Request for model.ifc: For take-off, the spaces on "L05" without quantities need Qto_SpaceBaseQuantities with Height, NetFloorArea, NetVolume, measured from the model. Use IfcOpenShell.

First a look at what the model holds.

```python
import ifcopenshell
import ifcopenshell.util.element
import ifcopenshell.util.unit

model = ifcopenshell.open("model.ifc")
print(model.schema)
for unit_type in ("LENGTHUNIT", "AREAUNIT", "VOLUMEUNIT"):
    print(unit_type, ifcopenshell.util.unit.calculate_unit_scale(model, unit_type))
storey = next(s for s in model.by_type("IfcBuildingStorey") if s.Name == "L05")
spaces = [e for e in ifcopenshell.util.element.get_decomposition(storey) if e.is_a("IfcSpace")]
for e in sorted(spaces, key=lambda e: e.id()):
    print(e.id(), e.is_a(), e.Name, list(ifcopenshell.util.element.get_psets(e, qtos_only=True)), sep=" | ")
```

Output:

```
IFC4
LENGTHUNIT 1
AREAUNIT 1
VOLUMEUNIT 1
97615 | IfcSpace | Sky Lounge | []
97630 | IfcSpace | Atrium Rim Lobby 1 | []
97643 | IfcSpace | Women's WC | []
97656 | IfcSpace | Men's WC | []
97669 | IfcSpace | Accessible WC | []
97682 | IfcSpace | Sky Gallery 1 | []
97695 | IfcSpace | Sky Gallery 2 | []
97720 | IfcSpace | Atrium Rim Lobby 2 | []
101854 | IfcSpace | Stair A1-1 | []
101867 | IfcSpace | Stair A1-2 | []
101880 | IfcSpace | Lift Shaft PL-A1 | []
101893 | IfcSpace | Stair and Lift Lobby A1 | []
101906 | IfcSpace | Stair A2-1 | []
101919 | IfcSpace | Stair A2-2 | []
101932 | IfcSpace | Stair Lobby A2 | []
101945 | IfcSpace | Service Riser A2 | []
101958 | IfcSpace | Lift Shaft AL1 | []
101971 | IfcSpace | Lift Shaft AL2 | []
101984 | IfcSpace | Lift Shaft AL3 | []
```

```python
import ifcopenshell
import ifcopenshell.api.pset
import ifcopenshell.geom
import ifcopenshell.util.element
import ifcopenshell.util.shape
import ifcopenshell.util.unit

model = ifcopenshell.open("model.ifc")
unit_scale = ifcopenshell.util.unit.calculate_unit_scale(model)
area_scale = ifcopenshell.util.unit.calculate_unit_scale(model, "AREAUNIT")
volume_scale = ifcopenshell.util.unit.calculate_unit_scale(model, "VOLUMEUNIT")
settings = ifcopenshell.geom.settings()

storey = next(s for s in model.by_type("IfcBuildingStorey") if s.Name == "L05")
spaces = [e for e in ifcopenshell.util.element.get_decomposition(storey) if e.is_a("IfcSpace")]

for e in sorted(spaces, key=lambda e: e.id()):
    if ifcopenshell.util.element.get_psets(e, qtos_only=True, should_inherit=False):
        continue
    # Geometry comes back in metres, in the element's own axes.
    shape = ifcopenshell.geom.create_shape(settings, e)
    values = {
        "Height": ifcopenshell.util.shape.get_z(shape.geometry) / unit_scale,
        "NetFloorArea": ifcopenshell.util.shape.get_footprint_area(shape.geometry) / area_scale,
        "NetVolume": ifcopenshell.util.shape.get_volume(shape.geometry) / volume_scale,
    }
    qto = ifcopenshell.api.pset.add_qto(model, product=e, name="Qto_SpaceBaseQuantities")
    ifcopenshell.api.pset.edit_qto(model, qto=qto, properties=values)
    print(e.id(), {k: round(v, 3) for k, v in values.items()})

model.write("model_rev.ifc")
```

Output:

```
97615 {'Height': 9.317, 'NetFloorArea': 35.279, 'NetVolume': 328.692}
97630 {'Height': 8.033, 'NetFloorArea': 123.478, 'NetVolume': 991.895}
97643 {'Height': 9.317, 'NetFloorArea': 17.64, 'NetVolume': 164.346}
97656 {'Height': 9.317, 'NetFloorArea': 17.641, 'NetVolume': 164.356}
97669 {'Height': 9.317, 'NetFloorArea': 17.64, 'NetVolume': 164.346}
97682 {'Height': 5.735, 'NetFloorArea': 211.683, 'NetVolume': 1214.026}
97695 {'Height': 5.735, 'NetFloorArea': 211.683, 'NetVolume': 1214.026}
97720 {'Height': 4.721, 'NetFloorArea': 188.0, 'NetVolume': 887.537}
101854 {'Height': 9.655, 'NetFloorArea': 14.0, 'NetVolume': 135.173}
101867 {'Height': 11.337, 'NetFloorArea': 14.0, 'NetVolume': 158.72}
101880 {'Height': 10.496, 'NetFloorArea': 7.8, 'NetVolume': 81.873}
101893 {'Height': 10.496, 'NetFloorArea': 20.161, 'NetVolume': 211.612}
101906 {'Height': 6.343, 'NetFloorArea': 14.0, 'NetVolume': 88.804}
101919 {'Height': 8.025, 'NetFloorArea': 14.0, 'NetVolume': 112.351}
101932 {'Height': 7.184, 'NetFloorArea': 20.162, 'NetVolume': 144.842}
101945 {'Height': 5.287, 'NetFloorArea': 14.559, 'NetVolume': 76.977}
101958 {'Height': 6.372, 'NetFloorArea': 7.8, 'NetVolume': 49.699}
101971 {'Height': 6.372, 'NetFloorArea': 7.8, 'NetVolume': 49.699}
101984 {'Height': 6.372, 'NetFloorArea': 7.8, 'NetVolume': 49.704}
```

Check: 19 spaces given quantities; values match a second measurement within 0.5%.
